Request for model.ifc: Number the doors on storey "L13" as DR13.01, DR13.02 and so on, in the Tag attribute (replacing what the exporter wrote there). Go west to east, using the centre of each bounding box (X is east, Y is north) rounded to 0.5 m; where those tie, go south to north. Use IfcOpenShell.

First a look at what the model holds.

```python
import ifcopenshell
import ifcopenshell.util.element
import ifcopenshell.util.placement

model = ifcopenshell.open("model.ifc")
print(model.schema)
storey = next(s for s in model.by_type("IfcBuildingStorey") if s.Name == "L13")
doors = [e for e in ifcopenshell.util.element.get_decomposition(storey) if e.is_a("IfcDoor")]
for e in sorted(doors, key=lambda e: e.id()):
    origin = ifcopenshell.util.placement.get_local_placement(e.ObjectPlacement)[:3, 3]
    print(e.id(), e.Tag, e.Name, origin.round(2) + 0.0, sep=" | ")
```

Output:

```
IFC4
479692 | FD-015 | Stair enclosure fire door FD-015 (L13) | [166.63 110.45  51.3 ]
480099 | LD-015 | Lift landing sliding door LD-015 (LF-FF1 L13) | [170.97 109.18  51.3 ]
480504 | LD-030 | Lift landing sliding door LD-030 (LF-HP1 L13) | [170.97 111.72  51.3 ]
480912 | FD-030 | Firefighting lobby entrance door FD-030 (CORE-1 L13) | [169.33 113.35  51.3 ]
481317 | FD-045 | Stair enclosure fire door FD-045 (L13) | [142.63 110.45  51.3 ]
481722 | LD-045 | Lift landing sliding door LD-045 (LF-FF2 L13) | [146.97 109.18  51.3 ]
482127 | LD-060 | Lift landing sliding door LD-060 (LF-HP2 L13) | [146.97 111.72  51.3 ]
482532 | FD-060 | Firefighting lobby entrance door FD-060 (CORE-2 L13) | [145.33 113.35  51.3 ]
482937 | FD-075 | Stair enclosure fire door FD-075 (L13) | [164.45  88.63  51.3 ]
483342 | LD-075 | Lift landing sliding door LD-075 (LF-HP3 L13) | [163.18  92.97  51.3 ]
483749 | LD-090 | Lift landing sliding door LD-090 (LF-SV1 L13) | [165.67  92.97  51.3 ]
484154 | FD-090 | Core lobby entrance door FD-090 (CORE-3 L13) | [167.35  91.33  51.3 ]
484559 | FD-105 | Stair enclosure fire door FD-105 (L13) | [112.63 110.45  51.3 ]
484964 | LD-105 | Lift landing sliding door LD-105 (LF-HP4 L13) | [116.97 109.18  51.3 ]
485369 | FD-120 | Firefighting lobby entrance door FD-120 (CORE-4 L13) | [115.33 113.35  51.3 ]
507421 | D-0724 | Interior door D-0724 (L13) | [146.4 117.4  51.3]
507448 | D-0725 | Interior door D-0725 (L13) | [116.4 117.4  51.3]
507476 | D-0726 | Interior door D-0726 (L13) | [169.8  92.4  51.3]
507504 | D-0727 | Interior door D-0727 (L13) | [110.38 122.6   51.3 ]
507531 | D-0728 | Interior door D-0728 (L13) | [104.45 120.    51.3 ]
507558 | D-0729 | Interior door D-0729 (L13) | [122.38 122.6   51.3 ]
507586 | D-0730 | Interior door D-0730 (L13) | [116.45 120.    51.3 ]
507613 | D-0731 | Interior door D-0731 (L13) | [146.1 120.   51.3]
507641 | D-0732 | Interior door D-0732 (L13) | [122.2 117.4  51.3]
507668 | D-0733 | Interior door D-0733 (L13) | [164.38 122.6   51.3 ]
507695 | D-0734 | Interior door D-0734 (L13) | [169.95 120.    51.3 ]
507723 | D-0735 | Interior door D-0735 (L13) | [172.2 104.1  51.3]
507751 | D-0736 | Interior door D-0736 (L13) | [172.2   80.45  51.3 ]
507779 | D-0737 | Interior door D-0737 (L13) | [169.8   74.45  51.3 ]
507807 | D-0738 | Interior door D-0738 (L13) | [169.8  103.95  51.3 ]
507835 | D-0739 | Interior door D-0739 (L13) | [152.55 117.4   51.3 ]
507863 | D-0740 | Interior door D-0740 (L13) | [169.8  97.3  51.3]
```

```python
import ifcopenshell
import ifcopenshell.geom
import ifcopenshell.util.element
import ifcopenshell.util.shape

model = ifcopenshell.open("model.ifc")
settings = ifcopenshell.geom.settings()
settings.set("use-world-coords", True)


def centre(element):
    shape = ifcopenshell.geom.create_shape(settings, element)
    return ifcopenshell.util.shape.get_bbox_centroid(shape.geometry)


storey = next(s for s in model.by_type("IfcBuildingStorey") if s.Name == "L13")
doors = [e for e in ifcopenshell.util.element.get_decomposition(storey) if e.is_a("IfcDoor")]

# Insertion points can sit at a corner or the storey origin, so sort by the geometry (in metres).
centres = {e: centre(e) for e in doors}
doors.sort(key=lambda e: (round(centres[e][0] / 0.5), centres[e][1]))

for i, e in enumerate(doors, start=1):
    number = f"DR13.{i:02d}"
    e.Tag = number
    print(e.id(), number)

model.write("model_v2.ifc")
```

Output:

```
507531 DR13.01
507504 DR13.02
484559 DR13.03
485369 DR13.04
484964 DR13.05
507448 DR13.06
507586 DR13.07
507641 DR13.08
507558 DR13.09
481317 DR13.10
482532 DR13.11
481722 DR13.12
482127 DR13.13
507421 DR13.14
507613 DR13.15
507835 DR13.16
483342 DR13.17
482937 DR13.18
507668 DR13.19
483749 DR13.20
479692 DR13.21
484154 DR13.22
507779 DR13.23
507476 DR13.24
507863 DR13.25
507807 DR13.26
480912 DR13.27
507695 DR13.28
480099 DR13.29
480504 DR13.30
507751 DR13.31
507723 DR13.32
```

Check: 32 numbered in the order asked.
